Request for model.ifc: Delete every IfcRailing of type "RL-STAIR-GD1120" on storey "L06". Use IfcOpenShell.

First a look at what the model holds.

```python
import ifcopenshell
import ifcopenshell.util.element

model = ifcopenshell.open("model.ifc")
print(model.schema)
storey = next(s for s in model.by_type("IfcBuildingStorey") if s.Name == "L06")
railings = [e for e in ifcopenshell.util.element.get_decomposition(storey) if e.is_a("IfcRailing")]
seen = {}
for e in railings:
    element_type = ifcopenshell.util.element.get_type(e)
    name = element_type.Name if element_type not in (None, e) else None
    seen[name] = seen.get(name, 0) + 1
for name, count in sorted(seen.items(), key=str):
    print(count, "x", name)
```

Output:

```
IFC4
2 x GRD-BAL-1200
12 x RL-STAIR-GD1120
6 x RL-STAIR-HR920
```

```python
import ifcopenshell
import ifcopenshell.api.root
import ifcopenshell.util.element

model = ifcopenshell.open("model.ifc")

storey = next(s for s in model.by_type("IfcBuildingStorey") if s.Name == "L06")
railings = [e for e in ifcopenshell.util.element.get_decomposition(storey) if e.is_a("IfcRailing")]
targets = [e for e in railings if (t := ifcopenshell.util.element.get_type(e)) not in (None, e) and t.Name == "RL-STAIR-GD1120"]

for e in targets:
    ifcopenshell.api.root.remove_product(model, product=e)
print(len(targets), "removed")

model.write("model_edited.ifc")
```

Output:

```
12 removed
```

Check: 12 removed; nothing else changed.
